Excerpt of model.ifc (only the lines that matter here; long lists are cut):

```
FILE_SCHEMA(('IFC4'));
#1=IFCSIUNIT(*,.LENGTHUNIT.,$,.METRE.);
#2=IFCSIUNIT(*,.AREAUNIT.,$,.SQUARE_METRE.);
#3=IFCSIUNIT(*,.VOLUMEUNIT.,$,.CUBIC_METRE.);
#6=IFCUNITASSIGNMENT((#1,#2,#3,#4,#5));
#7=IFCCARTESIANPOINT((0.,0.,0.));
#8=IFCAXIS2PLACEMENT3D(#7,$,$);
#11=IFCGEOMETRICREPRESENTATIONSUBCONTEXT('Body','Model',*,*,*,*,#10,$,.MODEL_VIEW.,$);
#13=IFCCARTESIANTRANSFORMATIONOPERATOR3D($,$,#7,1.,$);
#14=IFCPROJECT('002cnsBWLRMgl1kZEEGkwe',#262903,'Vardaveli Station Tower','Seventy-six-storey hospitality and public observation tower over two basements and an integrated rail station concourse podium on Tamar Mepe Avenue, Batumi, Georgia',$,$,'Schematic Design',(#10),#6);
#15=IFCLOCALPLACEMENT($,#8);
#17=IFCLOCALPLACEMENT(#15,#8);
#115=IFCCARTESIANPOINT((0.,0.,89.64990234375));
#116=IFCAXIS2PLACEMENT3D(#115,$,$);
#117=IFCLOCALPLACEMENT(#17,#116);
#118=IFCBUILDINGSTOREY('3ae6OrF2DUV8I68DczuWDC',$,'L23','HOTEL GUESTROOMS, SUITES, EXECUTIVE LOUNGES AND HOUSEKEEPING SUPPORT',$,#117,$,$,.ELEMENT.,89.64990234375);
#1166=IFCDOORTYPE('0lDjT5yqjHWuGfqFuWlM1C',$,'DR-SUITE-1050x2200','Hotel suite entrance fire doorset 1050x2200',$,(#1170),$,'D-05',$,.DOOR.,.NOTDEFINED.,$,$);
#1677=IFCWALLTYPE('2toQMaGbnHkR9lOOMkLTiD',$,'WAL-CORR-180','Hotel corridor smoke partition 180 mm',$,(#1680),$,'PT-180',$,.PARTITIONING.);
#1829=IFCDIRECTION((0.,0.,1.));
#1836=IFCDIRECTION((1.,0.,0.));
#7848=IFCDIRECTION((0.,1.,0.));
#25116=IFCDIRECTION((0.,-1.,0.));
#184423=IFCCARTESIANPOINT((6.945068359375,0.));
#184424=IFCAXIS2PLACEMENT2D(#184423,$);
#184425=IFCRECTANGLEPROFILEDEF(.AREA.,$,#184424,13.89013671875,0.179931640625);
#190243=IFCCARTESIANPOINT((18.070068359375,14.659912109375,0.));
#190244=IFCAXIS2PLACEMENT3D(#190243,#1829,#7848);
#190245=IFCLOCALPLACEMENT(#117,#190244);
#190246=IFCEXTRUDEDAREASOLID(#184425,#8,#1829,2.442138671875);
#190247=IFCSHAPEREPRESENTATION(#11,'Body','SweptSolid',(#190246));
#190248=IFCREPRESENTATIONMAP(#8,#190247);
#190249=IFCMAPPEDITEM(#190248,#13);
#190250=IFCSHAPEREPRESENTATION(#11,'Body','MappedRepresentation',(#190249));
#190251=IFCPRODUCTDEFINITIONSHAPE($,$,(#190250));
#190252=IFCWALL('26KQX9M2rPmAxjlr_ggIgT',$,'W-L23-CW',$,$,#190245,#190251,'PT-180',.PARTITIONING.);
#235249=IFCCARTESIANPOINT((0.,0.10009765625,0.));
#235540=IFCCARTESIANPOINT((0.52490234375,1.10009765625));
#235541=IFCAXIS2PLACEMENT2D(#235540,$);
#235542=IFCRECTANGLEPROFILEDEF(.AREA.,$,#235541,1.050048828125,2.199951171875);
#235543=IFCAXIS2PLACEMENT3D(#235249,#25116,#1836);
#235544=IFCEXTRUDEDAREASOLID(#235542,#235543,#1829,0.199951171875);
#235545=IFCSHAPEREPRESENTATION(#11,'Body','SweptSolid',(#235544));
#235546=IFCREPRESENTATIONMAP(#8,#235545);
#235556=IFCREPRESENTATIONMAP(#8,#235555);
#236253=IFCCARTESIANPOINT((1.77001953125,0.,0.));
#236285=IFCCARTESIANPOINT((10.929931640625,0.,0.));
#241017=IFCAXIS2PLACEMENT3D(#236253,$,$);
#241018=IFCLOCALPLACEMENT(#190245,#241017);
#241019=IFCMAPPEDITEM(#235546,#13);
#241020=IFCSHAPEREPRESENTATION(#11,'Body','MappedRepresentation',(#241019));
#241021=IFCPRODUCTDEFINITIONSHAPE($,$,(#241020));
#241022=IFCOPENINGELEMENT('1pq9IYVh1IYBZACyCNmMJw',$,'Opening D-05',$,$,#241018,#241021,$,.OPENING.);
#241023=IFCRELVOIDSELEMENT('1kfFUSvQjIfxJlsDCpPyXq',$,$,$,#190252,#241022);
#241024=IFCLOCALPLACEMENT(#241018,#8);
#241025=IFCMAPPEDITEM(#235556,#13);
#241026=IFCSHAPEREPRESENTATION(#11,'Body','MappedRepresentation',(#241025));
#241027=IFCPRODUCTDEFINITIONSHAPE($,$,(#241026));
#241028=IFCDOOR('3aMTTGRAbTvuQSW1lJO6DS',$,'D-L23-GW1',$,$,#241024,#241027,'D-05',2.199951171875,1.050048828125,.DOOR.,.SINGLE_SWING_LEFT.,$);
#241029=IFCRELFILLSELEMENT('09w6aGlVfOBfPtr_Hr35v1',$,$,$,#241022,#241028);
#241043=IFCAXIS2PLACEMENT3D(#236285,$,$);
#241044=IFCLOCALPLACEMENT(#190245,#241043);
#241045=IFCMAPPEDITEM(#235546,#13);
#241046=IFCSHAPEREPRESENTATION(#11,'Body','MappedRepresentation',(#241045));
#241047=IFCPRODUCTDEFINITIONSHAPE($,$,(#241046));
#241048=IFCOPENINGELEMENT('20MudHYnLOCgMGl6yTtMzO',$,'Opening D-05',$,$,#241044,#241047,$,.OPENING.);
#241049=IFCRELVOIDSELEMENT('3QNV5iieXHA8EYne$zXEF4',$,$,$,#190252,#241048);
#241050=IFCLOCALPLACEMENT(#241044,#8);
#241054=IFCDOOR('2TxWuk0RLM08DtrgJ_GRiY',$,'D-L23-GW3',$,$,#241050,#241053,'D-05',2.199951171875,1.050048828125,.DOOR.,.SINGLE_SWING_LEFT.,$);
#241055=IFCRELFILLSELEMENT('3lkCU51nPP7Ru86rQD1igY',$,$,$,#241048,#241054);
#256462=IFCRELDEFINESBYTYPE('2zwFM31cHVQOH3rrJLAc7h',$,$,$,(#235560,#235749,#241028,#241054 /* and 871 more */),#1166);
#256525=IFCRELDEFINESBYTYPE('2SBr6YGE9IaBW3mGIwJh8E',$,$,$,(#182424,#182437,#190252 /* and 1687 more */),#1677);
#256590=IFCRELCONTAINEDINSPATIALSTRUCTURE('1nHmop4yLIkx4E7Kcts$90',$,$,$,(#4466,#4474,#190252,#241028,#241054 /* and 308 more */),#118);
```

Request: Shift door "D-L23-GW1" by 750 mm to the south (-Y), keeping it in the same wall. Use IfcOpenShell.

```python
import ifcopenshell
import ifcopenshell.api.geometry
import ifcopenshell.util.placement

model = ifcopenshell.open("model.ifc")

door = model.by_id(241028)
opening = door.FillsVoids[0].RelatingOpeningElement
wall = opening.VoidsElements[0].RelatingBuildingElement

wall_matrix = ifcopenshell.util.placement.get_local_placement(wall.ObjectPlacement)
shift = wall_matrix[:3, 0] * -0.75
before = ifcopenshell.util.placement.get_local_placement(door.ObjectPlacement)[:3, 3].copy()

# The door is placed relative to its opening, so it follows when the opening moves.
matrix = ifcopenshell.util.placement.get_local_placement(opening.ObjectPlacement)
matrix[:3, 3] += shift
ifcopenshell.api.geometry.edit_object_placement(
    model, product=opening, matrix=matrix, is_si=False, should_transform_children=True
)

after = ifcopenshell.util.placement.get_local_placement(door.ObjectPlacement)[:3, 3]
print("door moved by", (after - before).round(3) + 0.0)

model.write("model_edited.ifc")
```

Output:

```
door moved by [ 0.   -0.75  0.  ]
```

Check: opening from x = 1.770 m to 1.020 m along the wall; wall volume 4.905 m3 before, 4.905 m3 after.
